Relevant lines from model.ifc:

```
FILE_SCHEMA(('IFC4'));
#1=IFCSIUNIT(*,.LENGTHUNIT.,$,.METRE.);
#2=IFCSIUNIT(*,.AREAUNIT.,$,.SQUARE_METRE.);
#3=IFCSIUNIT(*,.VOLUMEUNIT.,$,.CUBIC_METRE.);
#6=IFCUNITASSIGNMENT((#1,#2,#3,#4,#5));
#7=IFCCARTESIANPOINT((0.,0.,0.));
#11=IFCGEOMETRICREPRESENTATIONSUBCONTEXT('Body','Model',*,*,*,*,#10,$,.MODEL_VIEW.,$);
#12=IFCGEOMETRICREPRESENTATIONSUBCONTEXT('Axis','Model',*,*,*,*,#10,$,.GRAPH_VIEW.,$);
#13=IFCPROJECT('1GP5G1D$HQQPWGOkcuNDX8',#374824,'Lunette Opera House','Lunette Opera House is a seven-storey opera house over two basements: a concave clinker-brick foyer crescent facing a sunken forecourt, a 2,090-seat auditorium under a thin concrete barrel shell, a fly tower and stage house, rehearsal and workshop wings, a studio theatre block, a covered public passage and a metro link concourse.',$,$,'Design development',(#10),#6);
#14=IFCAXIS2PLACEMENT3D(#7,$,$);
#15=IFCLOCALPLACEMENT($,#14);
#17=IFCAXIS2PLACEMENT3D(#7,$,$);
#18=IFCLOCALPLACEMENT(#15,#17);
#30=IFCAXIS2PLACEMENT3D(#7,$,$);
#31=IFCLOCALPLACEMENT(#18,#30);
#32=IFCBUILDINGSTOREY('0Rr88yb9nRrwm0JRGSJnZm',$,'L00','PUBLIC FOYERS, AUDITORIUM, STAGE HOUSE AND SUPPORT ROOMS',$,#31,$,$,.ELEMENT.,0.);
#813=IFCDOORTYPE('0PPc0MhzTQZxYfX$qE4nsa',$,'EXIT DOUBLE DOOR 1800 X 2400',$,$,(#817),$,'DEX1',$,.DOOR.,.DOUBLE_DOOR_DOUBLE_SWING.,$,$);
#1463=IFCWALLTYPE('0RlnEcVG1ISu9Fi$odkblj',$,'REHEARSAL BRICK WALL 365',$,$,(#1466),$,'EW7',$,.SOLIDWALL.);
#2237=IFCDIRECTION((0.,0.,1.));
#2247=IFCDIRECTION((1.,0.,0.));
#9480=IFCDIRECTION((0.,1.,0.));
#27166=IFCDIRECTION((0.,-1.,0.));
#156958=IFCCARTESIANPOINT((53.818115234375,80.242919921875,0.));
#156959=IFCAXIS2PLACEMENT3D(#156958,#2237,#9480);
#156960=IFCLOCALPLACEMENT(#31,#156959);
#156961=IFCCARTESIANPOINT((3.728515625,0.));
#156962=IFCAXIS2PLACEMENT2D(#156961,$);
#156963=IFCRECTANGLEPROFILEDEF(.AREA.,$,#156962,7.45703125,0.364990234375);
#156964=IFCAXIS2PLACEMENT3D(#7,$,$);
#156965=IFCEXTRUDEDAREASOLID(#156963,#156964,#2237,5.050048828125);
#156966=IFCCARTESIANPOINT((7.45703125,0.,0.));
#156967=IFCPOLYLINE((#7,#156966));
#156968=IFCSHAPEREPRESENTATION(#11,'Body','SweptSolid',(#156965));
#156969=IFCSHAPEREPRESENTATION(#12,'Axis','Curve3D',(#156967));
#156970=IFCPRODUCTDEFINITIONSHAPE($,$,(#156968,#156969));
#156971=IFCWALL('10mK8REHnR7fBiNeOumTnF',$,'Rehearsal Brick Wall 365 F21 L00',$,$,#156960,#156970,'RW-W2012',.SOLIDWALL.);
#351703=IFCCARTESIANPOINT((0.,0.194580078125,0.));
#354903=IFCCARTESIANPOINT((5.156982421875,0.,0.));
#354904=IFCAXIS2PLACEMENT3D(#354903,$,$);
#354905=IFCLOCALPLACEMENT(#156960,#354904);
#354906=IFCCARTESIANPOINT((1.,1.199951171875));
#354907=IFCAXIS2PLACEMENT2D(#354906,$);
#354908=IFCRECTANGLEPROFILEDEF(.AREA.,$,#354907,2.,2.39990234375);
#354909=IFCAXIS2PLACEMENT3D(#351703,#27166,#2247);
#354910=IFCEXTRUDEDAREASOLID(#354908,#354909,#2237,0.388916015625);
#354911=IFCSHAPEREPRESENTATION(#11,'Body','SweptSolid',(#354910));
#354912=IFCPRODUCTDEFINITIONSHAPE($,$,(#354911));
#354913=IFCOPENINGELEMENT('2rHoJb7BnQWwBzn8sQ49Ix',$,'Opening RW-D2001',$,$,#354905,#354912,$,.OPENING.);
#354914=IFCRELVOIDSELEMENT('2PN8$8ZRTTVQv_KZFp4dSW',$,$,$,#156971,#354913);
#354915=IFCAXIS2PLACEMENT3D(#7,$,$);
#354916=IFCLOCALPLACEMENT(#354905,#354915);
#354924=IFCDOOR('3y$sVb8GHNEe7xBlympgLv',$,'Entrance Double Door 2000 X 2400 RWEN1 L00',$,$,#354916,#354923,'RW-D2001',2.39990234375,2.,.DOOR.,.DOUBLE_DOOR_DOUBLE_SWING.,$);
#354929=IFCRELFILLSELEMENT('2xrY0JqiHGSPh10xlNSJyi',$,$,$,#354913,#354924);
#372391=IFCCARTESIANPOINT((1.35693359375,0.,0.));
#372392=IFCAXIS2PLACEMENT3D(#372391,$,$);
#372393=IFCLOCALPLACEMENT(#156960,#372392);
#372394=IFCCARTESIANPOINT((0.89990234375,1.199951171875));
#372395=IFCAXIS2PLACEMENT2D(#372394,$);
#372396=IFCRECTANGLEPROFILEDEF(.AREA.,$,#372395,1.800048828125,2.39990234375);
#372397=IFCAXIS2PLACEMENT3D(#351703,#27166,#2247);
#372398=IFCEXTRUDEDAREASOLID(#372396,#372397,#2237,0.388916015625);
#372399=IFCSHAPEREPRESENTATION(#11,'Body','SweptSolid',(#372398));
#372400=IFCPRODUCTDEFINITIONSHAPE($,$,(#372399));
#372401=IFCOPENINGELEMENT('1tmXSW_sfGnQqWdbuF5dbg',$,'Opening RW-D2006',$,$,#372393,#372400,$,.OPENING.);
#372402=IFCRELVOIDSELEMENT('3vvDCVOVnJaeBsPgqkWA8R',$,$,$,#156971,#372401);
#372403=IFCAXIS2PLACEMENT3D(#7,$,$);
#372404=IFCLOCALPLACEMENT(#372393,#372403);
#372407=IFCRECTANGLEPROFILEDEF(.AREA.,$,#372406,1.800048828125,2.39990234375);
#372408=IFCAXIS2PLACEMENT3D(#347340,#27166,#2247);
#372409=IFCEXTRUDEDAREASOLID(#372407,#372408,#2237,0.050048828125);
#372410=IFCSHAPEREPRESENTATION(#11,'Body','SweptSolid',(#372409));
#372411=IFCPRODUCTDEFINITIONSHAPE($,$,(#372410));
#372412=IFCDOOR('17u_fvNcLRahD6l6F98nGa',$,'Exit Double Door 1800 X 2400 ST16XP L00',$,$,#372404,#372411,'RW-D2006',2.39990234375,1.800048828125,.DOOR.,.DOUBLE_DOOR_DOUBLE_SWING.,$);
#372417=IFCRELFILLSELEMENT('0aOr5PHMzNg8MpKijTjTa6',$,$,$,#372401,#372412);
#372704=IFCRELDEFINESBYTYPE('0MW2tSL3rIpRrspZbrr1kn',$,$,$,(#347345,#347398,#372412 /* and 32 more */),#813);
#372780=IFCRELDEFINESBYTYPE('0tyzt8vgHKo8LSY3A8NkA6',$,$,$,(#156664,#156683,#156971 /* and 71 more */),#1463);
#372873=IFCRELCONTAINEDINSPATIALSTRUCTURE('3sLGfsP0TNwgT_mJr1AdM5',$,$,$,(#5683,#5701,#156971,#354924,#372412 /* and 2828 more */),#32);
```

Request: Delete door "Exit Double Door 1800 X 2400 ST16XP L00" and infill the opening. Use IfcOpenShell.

```python
import ifcopenshell
import ifcopenshell.api.feature
import ifcopenshell.api.root
import ifcopenshell.geom
import ifcopenshell.util.shape

model = ifcopenshell.open("model.ifc")
settings = ifcopenshell.geom.settings()


def volume(element):
    """Net volume in cubic metres, openings subtracted."""
    shape = ifcopenshell.geom.create_shape(settings, element)
    return ifcopenshell.util.shape.get_volume(shape.geometry)


door = model.by_id(372412)
opening = door.FillsVoids[0].RelatingOpeningElement
wall = opening.VoidsElements[0].RelatingBuildingElement
before = volume(wall)

ifcopenshell.api.root.remove_product(model, product=door)
ifcopenshell.api.feature.remove_feature(model, feature=opening)

after = volume(wall)

print(f"wall volume {before:.3f} -> {after:.3f} m3")

model.write("model_updated.ifc")
```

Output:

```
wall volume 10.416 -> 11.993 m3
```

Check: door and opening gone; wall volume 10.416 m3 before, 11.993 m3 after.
